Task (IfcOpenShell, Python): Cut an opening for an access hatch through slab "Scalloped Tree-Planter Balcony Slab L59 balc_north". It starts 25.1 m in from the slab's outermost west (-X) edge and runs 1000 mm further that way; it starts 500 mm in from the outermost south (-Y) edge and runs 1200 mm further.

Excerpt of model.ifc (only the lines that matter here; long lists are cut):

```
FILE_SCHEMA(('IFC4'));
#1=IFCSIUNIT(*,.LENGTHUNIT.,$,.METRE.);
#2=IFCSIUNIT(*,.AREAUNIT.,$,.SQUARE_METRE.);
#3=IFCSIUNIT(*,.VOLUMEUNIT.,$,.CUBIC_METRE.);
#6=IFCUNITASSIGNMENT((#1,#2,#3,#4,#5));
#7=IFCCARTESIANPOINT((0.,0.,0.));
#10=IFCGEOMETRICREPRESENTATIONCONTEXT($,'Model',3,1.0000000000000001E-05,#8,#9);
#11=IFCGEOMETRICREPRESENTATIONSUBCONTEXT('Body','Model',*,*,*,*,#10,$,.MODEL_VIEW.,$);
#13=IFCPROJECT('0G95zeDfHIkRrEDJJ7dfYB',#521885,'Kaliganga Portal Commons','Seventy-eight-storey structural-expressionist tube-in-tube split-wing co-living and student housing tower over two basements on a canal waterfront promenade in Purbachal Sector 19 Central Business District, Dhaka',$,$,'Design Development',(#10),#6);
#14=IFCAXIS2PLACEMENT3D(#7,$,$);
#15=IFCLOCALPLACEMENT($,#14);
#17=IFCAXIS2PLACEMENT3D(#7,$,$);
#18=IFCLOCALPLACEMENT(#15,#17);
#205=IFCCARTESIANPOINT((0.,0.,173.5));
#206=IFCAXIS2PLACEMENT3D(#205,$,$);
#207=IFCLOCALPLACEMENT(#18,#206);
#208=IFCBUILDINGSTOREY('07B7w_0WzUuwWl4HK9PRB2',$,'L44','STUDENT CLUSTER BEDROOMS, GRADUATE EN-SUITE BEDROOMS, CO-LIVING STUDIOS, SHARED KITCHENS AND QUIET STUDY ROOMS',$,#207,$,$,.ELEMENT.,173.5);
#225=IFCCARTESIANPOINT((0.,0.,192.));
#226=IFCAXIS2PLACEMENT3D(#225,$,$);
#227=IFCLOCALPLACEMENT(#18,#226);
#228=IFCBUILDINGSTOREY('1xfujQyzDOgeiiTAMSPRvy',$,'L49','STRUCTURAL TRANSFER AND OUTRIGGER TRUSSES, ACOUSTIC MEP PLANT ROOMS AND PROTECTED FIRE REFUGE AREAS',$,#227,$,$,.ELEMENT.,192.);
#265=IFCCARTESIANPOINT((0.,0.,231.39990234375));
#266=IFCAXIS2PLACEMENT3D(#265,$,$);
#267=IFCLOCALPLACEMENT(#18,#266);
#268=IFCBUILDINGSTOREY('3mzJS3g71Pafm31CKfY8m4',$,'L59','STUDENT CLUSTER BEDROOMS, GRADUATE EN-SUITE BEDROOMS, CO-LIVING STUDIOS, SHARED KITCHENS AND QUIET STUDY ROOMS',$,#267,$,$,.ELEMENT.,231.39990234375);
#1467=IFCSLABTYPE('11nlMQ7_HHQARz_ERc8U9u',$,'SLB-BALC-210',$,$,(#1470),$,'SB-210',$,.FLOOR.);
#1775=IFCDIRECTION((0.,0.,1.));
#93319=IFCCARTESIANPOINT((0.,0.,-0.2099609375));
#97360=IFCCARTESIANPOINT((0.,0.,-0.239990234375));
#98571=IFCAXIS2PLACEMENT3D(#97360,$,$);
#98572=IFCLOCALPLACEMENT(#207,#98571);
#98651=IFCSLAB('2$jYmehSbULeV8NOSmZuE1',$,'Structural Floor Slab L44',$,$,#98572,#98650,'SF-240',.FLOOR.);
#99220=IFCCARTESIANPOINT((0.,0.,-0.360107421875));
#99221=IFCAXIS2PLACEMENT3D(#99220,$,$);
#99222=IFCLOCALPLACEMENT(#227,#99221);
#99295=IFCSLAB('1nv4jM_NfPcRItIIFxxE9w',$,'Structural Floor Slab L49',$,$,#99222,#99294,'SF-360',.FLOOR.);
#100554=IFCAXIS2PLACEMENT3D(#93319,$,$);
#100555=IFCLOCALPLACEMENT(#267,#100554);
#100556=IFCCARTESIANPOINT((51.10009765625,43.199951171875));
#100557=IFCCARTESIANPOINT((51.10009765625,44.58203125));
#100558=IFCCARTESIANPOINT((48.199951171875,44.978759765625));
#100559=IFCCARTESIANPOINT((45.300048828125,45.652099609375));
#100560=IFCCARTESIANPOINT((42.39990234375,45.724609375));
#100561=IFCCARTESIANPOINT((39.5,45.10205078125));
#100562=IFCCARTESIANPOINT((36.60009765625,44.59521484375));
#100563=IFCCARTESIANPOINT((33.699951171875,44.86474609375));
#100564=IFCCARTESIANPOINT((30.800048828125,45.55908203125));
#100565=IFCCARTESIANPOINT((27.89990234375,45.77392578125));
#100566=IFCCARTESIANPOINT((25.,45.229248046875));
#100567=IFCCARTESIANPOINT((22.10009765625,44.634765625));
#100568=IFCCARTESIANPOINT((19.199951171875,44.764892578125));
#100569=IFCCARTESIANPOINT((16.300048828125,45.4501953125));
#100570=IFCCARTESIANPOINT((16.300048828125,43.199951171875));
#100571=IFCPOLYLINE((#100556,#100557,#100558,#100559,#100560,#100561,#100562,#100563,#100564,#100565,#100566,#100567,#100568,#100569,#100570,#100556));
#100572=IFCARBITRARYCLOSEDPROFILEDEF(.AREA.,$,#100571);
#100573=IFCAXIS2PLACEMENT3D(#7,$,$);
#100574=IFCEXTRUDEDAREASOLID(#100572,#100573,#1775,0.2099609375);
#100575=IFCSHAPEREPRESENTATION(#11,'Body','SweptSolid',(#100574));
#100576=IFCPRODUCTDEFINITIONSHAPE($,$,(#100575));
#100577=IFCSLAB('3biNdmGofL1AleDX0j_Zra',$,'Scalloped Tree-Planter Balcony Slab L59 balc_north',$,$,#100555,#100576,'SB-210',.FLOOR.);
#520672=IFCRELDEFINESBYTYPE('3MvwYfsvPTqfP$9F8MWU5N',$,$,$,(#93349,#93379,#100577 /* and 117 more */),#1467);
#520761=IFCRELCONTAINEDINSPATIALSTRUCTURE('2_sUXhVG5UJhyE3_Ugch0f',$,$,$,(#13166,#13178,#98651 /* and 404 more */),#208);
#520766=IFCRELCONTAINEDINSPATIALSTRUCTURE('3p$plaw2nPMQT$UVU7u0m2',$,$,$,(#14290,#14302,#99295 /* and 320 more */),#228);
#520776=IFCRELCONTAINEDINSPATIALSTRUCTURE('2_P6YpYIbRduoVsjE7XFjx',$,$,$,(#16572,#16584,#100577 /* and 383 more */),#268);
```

```python
import numpy as np
import ifcopenshell
import ifcopenshell.api.feature
import ifcopenshell.api.geometry
import ifcopenshell.api.root
import ifcopenshell.geom
import ifcopenshell.util.placement
import ifcopenshell.util.representation
import ifcopenshell.util.shape
import ifcopenshell.util.unit

model = ifcopenshell.open("model.ifc")
unit_scale = ifcopenshell.util.unit.calculate_unit_scale(model)
settings = ifcopenshell.geom.settings()


def volume(element):
    """Net volume in cubic metres, openings subtracted."""
    shape = ifcopenshell.geom.create_shape(settings, element)
    return ifcopenshell.util.shape.get_volume(shape.geometry)


slab = model.by_guid("3biNdmGofL1AleDX0j_Zra")
before = volume(slab)

# Extent in the slab's own axes, in metres. The edges named are its -X and -Y sides.
slab_shape = ifcopenshell.geom.create_shape(settings, slab)
vertices = ifcopenshell.util.shape.get_vertices(slab_shape.geometry)
x_min, y_min, bottom = vertices.min(axis=0)
top = vertices[:, 2].max()

opening = ifcopenshell.api.root.create_entity(model, ifc_class="IfcOpeningElement", name="Access hatch opening", predefined_type="OPENING")
context = ifcopenshell.util.representation.get_context(model, "Model", "Body", "MODEL_VIEW")
width, depth = 1, 1.2
outline = [(0.0, 0.0), (width, 0.0), (width, depth), (0.0, depth), (0.0, 0.0)]
# Overshoot both faces by 50 mm so the cut is clean.
shape = ifcopenshell.api.geometry.add_slab_representation(
    model, context=context, depth=top - bottom + 0.1, polyline=outline
)
ifcopenshell.api.geometry.assign_representation(model, product=opening, representation=shape)

matrix = ifcopenshell.util.placement.get_local_placement(slab.ObjectPlacement)
matrix[:, 3] = matrix @ np.append(np.array([x_min + 25.1, y_min + 0.5, bottom - 0.05]) / unit_scale, 1.0)
ifcopenshell.api.geometry.edit_object_placement(model, product=opening, matrix=matrix, is_si=False)
ifcopenshell.api.feature.add_feature(model, feature=opening, element=slab)

after = volume(slab)

print(f"slab volume {before:.3f} -> {after:.3f} m3")

model.write("model_rev.ifc")
```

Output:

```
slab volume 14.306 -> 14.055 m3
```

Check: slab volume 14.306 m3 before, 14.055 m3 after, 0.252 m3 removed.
